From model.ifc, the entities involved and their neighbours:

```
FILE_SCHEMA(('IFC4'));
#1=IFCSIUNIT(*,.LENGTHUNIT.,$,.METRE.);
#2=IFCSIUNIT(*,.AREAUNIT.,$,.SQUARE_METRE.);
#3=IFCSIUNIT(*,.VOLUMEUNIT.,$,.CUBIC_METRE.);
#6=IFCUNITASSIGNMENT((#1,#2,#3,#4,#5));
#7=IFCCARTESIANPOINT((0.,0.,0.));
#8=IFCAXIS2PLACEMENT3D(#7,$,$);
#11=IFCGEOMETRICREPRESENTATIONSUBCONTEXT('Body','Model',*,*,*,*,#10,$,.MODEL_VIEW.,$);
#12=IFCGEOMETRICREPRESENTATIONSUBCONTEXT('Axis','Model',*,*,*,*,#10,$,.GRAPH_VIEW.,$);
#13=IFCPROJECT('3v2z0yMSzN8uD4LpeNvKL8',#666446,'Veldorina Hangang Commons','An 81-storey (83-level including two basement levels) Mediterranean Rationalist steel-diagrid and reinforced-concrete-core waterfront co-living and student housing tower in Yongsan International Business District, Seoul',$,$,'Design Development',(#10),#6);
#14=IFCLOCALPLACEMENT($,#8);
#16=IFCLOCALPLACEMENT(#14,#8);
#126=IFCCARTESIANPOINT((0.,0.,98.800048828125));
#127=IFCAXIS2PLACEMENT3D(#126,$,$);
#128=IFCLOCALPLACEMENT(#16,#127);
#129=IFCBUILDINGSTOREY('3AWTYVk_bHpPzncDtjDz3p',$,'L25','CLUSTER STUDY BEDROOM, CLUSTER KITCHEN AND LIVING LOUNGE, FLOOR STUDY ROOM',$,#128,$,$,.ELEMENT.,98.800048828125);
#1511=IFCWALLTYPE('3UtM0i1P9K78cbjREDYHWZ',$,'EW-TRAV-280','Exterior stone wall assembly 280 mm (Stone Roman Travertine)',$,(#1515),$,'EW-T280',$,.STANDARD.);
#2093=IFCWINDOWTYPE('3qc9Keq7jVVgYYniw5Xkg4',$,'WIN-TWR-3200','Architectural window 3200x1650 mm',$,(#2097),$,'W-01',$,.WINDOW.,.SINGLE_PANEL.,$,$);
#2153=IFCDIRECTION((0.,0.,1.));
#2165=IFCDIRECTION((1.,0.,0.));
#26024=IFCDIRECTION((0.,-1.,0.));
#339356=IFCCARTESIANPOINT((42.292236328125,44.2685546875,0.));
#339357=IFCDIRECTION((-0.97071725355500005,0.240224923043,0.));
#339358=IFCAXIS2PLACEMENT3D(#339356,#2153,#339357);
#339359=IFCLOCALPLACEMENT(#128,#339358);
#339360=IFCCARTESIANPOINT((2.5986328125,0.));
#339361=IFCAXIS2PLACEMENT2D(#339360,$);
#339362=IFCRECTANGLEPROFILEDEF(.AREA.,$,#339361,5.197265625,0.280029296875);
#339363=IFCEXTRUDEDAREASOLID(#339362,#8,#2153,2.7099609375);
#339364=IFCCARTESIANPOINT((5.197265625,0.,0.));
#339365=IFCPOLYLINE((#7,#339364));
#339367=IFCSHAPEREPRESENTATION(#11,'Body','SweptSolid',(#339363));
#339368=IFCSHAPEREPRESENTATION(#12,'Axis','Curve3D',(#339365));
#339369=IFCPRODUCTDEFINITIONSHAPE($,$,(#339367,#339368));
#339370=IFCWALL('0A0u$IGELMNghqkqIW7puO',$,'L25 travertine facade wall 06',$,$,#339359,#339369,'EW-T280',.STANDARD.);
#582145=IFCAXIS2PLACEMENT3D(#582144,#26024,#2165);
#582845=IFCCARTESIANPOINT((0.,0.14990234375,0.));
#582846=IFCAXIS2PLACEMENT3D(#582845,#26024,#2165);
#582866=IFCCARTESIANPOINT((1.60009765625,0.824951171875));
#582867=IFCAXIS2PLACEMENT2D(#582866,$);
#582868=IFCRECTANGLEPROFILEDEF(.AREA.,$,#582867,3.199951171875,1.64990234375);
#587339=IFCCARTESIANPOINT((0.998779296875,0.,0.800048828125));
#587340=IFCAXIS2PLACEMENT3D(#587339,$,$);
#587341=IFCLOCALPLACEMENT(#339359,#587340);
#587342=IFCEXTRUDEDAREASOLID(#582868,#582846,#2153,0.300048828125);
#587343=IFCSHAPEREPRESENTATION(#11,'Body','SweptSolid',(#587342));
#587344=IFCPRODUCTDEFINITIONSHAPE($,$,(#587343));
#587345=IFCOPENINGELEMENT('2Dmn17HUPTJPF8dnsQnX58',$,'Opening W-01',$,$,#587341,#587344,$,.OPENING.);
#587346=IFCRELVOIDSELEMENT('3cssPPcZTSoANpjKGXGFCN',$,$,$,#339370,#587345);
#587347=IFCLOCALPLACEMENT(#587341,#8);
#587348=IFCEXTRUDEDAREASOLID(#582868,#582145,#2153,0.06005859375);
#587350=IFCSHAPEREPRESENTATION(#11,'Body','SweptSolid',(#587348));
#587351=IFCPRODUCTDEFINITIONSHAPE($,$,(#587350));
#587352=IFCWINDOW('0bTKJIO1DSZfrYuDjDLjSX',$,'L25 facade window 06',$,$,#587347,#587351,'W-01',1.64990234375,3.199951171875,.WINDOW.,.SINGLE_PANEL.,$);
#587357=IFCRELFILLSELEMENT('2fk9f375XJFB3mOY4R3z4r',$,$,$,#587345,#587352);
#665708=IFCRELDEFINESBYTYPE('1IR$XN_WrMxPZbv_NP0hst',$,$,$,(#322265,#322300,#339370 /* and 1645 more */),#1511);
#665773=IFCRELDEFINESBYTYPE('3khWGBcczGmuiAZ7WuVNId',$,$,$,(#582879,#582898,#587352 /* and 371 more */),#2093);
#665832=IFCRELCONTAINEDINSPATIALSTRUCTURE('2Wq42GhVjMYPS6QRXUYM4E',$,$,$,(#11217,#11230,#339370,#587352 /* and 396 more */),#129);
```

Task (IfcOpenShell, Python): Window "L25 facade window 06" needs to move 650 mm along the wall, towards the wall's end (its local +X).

```python
import ifcopenshell
import ifcopenshell.api.geometry
import ifcopenshell.util.placement
import ifcopenshell.util.unit

model = ifcopenshell.open("model.ifc")
unit_scale = ifcopenshell.util.unit.calculate_unit_scale(model)

window = model.by_id(587352)
opening = window.FillsVoids[0].RelatingOpeningElement
wall = opening.VoidsElements[0].RelatingBuildingElement

wall_matrix = ifcopenshell.util.placement.get_local_placement(wall.ObjectPlacement)
shift = wall_matrix[:3, 0] * 0.65 / unit_scale
before = ifcopenshell.util.placement.get_local_placement(window.ObjectPlacement)[:3, 3].copy()

# The window is placed relative to its opening, so it follows when the opening moves.
matrix = ifcopenshell.util.placement.get_local_placement(opening.ObjectPlacement)
matrix[:3, 3] += shift
ifcopenshell.api.geometry.edit_object_placement(
    model, product=opening, matrix=matrix, is_si=False, should_transform_children=True
)

after = ifcopenshell.util.placement.get_local_placement(window.ObjectPlacement)[:3, 3]
print("window moved by", (after - before).round(3) + 0.0)

model.write("model-out.ifc")
```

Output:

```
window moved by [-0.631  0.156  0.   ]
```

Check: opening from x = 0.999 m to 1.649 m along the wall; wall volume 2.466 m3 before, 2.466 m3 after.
